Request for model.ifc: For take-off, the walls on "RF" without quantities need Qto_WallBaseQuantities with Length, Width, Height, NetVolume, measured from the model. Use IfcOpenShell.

First a look at what the model holds.

```python
import ifcopenshell
import ifcopenshell.util.element
import ifcopenshell.util.unit

model = ifcopenshell.open("model.ifc")
print(model.schema)
for unit_type in ("LENGTHUNIT", "AREAUNIT", "VOLUMEUNIT"):
    print(unit_type, ifcopenshell.util.unit.calculate_unit_scale(model, unit_type))
storey = next(s for s in model.by_type("IfcBuildingStorey") if s.Name == "RF")
walls = [e for e in ifcopenshell.util.element.get_decomposition(storey) if e.is_a("IfcWall")]
for e in sorted(walls, key=lambda e: e.id()):
    print(e.id(), e.is_a(), e.Name, list(ifcopenshell.util.element.get_psets(e, qtos_only=True)), sep=" | ")
```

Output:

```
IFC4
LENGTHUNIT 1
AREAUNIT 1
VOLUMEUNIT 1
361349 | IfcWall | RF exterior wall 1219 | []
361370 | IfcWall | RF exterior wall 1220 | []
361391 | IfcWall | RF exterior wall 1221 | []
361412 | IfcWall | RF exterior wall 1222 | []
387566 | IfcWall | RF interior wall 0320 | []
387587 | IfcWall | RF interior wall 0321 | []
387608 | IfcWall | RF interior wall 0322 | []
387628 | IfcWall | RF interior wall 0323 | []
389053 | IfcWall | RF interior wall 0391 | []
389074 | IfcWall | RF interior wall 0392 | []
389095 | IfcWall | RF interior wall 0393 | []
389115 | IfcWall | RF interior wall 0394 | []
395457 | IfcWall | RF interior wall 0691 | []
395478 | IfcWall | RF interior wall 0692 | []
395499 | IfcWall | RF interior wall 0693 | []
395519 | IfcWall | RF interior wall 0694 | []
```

```python
import ifcopenshell
import ifcopenshell.api.pset
import ifcopenshell.geom
import ifcopenshell.util.element
import ifcopenshell.util.shape
import ifcopenshell.util.unit

model = ifcopenshell.open("model.ifc")
unit_scale = ifcopenshell.util.unit.calculate_unit_scale(model)
volume_scale = ifcopenshell.util.unit.calculate_unit_scale(model, "VOLUMEUNIT")
settings = ifcopenshell.geom.settings()

storey = next(s for s in model.by_type("IfcBuildingStorey") if s.Name == "RF")
walls = [e for e in ifcopenshell.util.element.get_decomposition(storey) if e.is_a("IfcWall")]

for e in sorted(walls, key=lambda e: e.id()):
    if ifcopenshell.util.element.get_psets(e, qtos_only=True, should_inherit=False):
        continue
    # Geometry comes back in metres, in the element's own axes.
    shape = ifcopenshell.geom.create_shape(settings, e)
    values = {
        "Length": ifcopenshell.util.shape.get_x(shape.geometry) / unit_scale,
        "Width": ifcopenshell.util.shape.get_y(shape.geometry) / unit_scale,
        "Height": ifcopenshell.util.shape.get_z(shape.geometry) / unit_scale,
        "NetVolume": ifcopenshell.util.shape.get_volume(shape.geometry) / volume_scale,
    }
    qto = ifcopenshell.api.pset.add_qto(model, product=e, name="Qto_WallBaseQuantities")
    ifcopenshell.api.pset.edit_qto(model, qto=qto, properties=values)
    print(e.id(), {k: round(v, 3) for k, v in values.items()})

model.write("model-out.ifc")
```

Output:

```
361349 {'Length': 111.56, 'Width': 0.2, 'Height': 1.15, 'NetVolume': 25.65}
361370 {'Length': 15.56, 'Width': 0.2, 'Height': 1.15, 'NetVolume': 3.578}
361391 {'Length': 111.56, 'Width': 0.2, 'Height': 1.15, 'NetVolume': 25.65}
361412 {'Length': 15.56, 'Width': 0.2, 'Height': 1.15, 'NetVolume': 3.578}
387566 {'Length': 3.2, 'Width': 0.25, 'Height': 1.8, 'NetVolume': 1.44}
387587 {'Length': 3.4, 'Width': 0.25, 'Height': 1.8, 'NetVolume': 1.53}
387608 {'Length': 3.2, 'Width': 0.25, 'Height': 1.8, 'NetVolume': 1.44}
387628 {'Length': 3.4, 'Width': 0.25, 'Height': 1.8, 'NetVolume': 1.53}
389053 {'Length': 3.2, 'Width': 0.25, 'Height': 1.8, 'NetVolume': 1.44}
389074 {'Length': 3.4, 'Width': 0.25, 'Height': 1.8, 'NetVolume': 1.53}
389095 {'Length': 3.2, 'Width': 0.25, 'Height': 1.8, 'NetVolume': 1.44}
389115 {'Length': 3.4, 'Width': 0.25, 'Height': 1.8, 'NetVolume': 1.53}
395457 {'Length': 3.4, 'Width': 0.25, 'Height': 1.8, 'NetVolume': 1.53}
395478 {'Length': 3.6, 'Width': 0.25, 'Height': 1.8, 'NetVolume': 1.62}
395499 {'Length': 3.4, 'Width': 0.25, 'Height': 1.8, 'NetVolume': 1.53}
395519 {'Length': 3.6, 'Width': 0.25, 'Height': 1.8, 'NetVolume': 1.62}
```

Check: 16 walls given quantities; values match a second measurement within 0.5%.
